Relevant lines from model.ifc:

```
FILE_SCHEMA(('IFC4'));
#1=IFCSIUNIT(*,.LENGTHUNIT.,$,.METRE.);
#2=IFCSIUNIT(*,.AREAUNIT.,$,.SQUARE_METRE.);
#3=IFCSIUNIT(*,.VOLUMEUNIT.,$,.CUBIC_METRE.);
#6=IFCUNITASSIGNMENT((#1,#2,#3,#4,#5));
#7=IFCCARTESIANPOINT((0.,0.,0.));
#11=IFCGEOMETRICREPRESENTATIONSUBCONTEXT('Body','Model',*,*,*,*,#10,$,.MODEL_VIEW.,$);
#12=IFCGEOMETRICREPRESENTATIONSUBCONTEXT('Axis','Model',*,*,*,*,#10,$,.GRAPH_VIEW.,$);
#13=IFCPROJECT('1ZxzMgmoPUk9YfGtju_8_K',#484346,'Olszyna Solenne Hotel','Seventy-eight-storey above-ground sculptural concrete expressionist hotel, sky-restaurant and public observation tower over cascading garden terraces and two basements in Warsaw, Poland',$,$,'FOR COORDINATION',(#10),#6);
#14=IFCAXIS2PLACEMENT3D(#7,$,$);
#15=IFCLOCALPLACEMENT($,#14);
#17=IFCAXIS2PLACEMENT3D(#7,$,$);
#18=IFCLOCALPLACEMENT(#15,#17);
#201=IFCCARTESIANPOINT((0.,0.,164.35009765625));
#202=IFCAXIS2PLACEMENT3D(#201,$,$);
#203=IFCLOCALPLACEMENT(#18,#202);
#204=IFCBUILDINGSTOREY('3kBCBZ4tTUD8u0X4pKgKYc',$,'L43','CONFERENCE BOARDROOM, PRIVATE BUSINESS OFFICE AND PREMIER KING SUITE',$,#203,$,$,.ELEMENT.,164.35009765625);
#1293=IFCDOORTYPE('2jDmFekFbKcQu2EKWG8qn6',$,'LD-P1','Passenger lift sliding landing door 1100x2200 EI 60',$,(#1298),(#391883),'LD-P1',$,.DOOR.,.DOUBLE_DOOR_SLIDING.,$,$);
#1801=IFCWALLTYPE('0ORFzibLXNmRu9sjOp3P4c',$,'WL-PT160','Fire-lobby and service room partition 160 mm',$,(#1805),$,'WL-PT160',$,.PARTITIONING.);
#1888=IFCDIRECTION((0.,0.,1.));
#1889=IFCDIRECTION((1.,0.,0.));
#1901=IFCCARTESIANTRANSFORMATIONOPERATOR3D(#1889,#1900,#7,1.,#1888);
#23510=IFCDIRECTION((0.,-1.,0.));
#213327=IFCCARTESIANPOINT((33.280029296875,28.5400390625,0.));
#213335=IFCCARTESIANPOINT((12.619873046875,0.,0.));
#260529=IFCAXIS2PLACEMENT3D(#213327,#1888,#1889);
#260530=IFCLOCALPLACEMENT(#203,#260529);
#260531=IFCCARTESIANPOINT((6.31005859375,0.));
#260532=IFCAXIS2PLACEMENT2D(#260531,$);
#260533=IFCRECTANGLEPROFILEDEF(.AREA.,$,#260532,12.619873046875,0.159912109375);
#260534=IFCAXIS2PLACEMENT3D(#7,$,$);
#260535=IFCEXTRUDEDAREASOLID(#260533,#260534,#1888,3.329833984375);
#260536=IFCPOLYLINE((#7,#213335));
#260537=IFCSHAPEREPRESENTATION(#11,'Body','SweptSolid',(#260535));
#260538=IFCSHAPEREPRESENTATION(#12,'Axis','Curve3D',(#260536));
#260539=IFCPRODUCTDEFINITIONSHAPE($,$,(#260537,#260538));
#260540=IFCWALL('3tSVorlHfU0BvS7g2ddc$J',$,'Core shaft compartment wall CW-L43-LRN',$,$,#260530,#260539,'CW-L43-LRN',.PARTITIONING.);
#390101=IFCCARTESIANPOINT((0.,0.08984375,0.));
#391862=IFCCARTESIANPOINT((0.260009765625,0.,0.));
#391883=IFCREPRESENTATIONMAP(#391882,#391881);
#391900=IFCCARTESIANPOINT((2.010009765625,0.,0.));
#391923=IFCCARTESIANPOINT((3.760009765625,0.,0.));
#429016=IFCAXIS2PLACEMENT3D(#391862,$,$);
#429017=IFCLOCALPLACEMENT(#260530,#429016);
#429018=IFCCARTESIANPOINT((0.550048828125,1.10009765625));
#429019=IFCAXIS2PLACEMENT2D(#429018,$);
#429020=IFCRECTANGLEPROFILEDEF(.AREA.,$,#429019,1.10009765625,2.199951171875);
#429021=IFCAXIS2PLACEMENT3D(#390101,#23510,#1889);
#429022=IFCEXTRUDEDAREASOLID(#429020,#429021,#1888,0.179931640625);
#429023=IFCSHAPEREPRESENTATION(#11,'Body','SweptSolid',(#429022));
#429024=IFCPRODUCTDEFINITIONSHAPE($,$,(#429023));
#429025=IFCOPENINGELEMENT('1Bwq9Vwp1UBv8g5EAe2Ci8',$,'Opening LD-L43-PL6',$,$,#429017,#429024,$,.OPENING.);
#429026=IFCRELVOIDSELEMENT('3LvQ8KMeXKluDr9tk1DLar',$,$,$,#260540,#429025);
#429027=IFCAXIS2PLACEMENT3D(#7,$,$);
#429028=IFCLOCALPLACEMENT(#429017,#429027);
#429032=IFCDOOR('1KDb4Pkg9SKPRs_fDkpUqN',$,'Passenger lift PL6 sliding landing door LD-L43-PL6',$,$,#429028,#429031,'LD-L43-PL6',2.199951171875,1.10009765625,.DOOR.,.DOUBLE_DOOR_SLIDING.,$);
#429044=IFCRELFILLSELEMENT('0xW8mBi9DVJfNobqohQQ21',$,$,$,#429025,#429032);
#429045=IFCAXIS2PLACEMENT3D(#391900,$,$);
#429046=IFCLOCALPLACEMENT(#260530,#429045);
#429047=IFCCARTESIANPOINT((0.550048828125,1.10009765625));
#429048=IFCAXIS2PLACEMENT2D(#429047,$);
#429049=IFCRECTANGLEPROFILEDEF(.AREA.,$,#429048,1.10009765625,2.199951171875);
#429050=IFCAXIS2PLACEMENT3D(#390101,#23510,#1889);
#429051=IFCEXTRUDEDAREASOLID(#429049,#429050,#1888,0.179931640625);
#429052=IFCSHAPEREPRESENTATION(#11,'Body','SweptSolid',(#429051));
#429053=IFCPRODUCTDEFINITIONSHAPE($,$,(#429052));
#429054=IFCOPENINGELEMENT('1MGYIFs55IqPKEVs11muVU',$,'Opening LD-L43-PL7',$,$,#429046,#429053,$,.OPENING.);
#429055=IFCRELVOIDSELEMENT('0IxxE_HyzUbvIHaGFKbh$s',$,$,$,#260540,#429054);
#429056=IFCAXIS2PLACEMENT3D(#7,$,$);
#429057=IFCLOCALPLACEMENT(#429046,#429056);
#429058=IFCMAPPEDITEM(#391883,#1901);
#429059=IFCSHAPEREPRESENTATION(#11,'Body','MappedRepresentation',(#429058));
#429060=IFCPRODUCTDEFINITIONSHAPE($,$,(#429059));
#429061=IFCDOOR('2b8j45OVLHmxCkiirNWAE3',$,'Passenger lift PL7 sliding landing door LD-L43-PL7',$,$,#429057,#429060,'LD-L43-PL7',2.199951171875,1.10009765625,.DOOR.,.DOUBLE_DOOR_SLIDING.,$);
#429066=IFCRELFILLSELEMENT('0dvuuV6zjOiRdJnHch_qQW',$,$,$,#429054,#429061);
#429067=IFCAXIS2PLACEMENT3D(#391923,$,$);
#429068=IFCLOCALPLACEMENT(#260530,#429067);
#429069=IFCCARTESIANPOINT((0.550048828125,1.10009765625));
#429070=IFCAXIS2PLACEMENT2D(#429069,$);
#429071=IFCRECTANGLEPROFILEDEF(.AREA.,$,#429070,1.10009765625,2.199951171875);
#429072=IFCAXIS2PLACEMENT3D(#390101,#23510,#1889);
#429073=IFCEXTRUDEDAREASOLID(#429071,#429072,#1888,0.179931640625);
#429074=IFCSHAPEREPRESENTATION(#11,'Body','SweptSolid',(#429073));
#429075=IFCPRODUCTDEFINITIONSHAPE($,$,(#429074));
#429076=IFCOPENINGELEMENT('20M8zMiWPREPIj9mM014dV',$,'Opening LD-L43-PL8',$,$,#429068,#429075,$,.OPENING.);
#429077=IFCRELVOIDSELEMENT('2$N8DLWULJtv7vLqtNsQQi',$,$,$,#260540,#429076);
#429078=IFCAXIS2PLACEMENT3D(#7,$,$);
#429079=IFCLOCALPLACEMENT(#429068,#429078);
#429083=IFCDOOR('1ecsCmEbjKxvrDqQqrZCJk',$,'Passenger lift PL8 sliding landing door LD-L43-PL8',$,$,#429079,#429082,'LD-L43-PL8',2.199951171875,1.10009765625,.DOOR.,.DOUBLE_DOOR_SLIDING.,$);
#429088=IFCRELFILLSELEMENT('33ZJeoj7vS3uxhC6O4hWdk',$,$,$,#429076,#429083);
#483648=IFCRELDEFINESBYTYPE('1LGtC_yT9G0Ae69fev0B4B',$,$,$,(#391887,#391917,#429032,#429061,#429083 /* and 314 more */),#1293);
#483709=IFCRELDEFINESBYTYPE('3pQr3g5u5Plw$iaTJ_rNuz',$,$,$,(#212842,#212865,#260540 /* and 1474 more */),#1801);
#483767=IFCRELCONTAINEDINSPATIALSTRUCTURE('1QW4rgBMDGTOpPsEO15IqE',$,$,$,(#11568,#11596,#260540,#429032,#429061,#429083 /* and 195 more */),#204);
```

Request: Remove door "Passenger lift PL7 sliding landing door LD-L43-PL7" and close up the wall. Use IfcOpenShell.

```python
import ifcopenshell
import ifcopenshell.api.feature
import ifcopenshell.api.root
import ifcopenshell.geom
import ifcopenshell.util.shape

model = ifcopenshell.open("model.ifc")
settings = ifcopenshell.geom.settings()


def volume(element):
    """Net volume in cubic metres, openings subtracted."""
    shape = ifcopenshell.geom.create_shape(settings, element)
    return ifcopenshell.util.shape.get_volume(shape.geometry)


door = model.by_id(429061)
opening = door.FillsVoids[0].RelatingOpeningElement
wall = opening.VoidsElements[0].RelatingBuildingElement
before = volume(wall)

ifcopenshell.api.root.remove_product(model, product=door)
ifcopenshell.api.feature.remove_feature(model, feature=opening)

after = volume(wall)

print(f"wall volume {before:.3f} -> {after:.3f} m3")

model.write("model_rev.ifc")
```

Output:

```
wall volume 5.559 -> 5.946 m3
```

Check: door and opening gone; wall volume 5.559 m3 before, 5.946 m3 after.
